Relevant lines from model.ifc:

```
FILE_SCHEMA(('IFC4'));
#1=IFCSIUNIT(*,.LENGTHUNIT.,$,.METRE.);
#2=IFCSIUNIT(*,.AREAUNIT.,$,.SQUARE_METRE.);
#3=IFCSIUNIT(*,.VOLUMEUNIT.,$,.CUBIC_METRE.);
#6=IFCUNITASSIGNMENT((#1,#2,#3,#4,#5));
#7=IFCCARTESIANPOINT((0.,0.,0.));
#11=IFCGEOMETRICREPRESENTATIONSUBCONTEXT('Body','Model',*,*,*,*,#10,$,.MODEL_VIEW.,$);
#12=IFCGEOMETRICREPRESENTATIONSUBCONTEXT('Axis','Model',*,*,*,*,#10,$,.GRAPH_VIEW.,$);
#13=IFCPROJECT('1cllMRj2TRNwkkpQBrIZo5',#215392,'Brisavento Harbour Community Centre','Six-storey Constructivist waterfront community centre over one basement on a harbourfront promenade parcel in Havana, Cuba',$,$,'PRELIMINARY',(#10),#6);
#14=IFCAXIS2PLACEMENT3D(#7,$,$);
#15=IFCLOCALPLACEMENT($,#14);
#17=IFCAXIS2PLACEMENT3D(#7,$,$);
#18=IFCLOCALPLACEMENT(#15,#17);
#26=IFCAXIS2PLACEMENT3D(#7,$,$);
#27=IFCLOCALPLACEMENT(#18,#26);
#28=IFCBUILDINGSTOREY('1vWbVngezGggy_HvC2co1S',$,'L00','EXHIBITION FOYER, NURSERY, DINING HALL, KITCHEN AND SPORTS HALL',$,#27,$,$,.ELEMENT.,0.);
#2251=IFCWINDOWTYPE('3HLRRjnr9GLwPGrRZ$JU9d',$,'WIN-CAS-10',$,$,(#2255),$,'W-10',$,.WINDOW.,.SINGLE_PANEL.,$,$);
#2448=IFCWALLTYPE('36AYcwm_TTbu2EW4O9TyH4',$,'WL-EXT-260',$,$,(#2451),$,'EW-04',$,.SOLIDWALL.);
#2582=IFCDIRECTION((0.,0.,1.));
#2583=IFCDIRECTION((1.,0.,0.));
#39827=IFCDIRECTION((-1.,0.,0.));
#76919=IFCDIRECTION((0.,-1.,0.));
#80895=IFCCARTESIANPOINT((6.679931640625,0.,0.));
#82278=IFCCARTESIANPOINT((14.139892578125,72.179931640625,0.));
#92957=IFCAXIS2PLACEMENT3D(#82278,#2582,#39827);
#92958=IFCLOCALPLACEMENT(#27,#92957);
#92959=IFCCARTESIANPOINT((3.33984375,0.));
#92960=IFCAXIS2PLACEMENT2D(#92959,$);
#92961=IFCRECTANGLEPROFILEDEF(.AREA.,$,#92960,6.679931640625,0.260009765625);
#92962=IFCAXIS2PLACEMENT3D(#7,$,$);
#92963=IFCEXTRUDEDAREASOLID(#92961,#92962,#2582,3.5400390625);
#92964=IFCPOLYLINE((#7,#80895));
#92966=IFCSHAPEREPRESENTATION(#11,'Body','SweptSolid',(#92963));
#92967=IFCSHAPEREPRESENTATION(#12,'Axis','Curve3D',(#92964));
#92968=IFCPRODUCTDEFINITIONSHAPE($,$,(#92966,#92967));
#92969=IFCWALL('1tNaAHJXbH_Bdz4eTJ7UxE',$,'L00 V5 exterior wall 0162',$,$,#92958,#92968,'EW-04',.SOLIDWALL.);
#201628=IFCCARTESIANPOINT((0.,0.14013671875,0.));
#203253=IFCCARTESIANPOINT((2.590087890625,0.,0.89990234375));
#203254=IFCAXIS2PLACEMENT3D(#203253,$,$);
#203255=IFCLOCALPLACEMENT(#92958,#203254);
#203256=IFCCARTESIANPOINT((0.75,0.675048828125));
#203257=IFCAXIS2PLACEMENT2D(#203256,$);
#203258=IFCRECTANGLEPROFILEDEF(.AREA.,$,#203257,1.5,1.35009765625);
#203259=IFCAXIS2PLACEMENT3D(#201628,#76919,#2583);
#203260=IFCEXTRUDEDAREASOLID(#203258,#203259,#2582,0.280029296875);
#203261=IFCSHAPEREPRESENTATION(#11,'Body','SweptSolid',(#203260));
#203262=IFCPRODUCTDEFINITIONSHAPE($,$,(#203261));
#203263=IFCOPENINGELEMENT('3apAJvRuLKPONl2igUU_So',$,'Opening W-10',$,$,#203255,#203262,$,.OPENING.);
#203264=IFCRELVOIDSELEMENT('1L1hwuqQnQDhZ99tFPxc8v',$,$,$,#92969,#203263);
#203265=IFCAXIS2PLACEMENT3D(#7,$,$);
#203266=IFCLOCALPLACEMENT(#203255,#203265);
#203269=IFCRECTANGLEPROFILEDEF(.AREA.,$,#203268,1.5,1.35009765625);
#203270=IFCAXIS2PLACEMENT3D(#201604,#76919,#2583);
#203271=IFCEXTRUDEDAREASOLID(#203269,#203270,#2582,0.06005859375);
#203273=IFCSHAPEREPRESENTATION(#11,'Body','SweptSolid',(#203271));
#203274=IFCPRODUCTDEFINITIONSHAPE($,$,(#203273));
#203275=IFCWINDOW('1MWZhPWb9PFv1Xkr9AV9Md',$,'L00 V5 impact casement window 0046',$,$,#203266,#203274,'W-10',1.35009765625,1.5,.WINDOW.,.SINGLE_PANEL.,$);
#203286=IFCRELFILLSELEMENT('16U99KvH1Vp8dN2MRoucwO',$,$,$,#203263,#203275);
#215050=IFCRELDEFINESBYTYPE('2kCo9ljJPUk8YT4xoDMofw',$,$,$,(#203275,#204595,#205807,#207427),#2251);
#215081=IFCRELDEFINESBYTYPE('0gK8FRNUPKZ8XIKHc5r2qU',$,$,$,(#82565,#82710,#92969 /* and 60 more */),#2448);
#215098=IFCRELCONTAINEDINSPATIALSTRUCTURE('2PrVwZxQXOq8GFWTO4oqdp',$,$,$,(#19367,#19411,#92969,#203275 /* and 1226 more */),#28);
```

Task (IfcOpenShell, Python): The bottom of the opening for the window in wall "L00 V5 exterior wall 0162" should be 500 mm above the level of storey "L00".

```python
import numpy as np
import ifcopenshell
import ifcopenshell.api.geometry
import ifcopenshell.geom
import ifcopenshell.util.element
import ifcopenshell.util.placement
import ifcopenshell.util.shape
import ifcopenshell.util.unit

model = ifcopenshell.open("model.ifc")
unit_scale = ifcopenshell.util.unit.calculate_unit_scale(model)

window = model.by_guid("1MWZhPWb9PFv1Xkr9AV9Md")
opening = window.FillsVoids[0].RelatingOpeningElement
storey = ifcopenshell.util.element.get_container(window, ifc_class="IfcBuildingStorey")
level = ifcopenshell.util.placement.get_local_placement(storey.ObjectPlacement)[2, 3]

# The opening's origin need not be at the sill, so measure its lowest point.
shape = ifcopenshell.geom.create_shape(ifcopenshell.geom.settings(), opening)
bottom = ifcopenshell.util.shape.get_shape_bottom_elevation(shape, shape.geometry) / unit_scale
dz = level + 0.5 - bottom

shift = np.array([0.0, 0.0, dz])
# The window is placed relative to its opening, so it follows when the opening moves.
matrix = ifcopenshell.util.placement.get_local_placement(opening.ObjectPlacement)
matrix[:3, 3] += shift
ifcopenshell.api.geometry.edit_object_placement(
    model, product=opening, matrix=matrix, is_si=False, should_transform_children=True
)

print(f"moved by {dz * unit_scale:+.3f} m")

model.write("model_edited.ifc")
```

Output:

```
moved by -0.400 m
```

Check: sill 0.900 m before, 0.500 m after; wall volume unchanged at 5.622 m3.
